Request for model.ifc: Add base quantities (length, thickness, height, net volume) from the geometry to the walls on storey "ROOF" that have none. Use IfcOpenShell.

First a look at what the model holds.

```python
import ifcopenshell
import ifcopenshell.util.element
import ifcopenshell.util.unit

model = ifcopenshell.open("model.ifc")
print(model.schema)
for unit_type in ("LENGTHUNIT", "AREAUNIT", "VOLUMEUNIT"):
    print(unit_type, ifcopenshell.util.unit.calculate_unit_scale(model, unit_type))
storey = next(s for s in model.by_type("IfcBuildingStorey") if s.Name == "ROOF")
walls = [e for e in ifcopenshell.util.element.get_decomposition(storey) if e.is_a("IfcWall")]
for e in sorted(walls, key=lambda e: e.id()):
    print(e.id(), e.is_a(), e.Name, list(ifcopenshell.util.element.get_psets(e, qtos_only=True)), sep=" | ")
```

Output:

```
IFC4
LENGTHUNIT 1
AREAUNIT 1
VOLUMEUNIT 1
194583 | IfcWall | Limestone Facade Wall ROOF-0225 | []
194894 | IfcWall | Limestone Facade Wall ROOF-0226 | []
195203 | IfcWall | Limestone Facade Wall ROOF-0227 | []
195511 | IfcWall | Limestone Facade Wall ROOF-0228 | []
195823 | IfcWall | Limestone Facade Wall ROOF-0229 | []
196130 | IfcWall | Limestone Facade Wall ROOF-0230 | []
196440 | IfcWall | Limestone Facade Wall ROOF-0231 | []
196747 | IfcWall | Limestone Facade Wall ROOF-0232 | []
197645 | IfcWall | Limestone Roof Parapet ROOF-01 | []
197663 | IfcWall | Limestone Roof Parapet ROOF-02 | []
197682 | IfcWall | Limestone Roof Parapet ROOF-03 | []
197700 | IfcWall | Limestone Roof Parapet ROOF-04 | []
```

```python
import ifcopenshell
import ifcopenshell.api.pset
import ifcopenshell.geom
import ifcopenshell.util.element
import ifcopenshell.util.shape
import ifcopenshell.util.unit

model = ifcopenshell.open("model.ifc")
unit_scale = ifcopenshell.util.unit.calculate_unit_scale(model)
volume_scale = ifcopenshell.util.unit.calculate_unit_scale(model, "VOLUMEUNIT")
settings = ifcopenshell.geom.settings()

storey = next(s for s in model.by_type("IfcBuildingStorey") if s.Name == "ROOF")
walls = [e for e in ifcopenshell.util.element.get_decomposition(storey) if e.is_a("IfcWall")]

for e in sorted(walls, key=lambda e: e.id()):
    if ifcopenshell.util.element.get_psets(e, qtos_only=True, should_inherit=False):
        continue
    # Geometry comes back in metres, in the element's own axes.
    shape = ifcopenshell.geom.create_shape(settings, e)
    values = {
        "Length": ifcopenshell.util.shape.get_x(shape.geometry) / unit_scale,
        "Width": ifcopenshell.util.shape.get_y(shape.geometry) / unit_scale,
        "Height": ifcopenshell.util.shape.get_z(shape.geometry) / unit_scale,
        "NetVolume": ifcopenshell.util.shape.get_volume(shape.geometry) / volume_scale,
    }
    qto = ifcopenshell.api.pset.add_qto(model, product=e, name="Qto_WallBaseQuantities")
    ifcopenshell.api.pset.edit_qto(model, qto=qto, properties=values)
    print(e.id(), {k: round(v, 3) for k, v in values.items()})

model.write("model_v2.ifc")
```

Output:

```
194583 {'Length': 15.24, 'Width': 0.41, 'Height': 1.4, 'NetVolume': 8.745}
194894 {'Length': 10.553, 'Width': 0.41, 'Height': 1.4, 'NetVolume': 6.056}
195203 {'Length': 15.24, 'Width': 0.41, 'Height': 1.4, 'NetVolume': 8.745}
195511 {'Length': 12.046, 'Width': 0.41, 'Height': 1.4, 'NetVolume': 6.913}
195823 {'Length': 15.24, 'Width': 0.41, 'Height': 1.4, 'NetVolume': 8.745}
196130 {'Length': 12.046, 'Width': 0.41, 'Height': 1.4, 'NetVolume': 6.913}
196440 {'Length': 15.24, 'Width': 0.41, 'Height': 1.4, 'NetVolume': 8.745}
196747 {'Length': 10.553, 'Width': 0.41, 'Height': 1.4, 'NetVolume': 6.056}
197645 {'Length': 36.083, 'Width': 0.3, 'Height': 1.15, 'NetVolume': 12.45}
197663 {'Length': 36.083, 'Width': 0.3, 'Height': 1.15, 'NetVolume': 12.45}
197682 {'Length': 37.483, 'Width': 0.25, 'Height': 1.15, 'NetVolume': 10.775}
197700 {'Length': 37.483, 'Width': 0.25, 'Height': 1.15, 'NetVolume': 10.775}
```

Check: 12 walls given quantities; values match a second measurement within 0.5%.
